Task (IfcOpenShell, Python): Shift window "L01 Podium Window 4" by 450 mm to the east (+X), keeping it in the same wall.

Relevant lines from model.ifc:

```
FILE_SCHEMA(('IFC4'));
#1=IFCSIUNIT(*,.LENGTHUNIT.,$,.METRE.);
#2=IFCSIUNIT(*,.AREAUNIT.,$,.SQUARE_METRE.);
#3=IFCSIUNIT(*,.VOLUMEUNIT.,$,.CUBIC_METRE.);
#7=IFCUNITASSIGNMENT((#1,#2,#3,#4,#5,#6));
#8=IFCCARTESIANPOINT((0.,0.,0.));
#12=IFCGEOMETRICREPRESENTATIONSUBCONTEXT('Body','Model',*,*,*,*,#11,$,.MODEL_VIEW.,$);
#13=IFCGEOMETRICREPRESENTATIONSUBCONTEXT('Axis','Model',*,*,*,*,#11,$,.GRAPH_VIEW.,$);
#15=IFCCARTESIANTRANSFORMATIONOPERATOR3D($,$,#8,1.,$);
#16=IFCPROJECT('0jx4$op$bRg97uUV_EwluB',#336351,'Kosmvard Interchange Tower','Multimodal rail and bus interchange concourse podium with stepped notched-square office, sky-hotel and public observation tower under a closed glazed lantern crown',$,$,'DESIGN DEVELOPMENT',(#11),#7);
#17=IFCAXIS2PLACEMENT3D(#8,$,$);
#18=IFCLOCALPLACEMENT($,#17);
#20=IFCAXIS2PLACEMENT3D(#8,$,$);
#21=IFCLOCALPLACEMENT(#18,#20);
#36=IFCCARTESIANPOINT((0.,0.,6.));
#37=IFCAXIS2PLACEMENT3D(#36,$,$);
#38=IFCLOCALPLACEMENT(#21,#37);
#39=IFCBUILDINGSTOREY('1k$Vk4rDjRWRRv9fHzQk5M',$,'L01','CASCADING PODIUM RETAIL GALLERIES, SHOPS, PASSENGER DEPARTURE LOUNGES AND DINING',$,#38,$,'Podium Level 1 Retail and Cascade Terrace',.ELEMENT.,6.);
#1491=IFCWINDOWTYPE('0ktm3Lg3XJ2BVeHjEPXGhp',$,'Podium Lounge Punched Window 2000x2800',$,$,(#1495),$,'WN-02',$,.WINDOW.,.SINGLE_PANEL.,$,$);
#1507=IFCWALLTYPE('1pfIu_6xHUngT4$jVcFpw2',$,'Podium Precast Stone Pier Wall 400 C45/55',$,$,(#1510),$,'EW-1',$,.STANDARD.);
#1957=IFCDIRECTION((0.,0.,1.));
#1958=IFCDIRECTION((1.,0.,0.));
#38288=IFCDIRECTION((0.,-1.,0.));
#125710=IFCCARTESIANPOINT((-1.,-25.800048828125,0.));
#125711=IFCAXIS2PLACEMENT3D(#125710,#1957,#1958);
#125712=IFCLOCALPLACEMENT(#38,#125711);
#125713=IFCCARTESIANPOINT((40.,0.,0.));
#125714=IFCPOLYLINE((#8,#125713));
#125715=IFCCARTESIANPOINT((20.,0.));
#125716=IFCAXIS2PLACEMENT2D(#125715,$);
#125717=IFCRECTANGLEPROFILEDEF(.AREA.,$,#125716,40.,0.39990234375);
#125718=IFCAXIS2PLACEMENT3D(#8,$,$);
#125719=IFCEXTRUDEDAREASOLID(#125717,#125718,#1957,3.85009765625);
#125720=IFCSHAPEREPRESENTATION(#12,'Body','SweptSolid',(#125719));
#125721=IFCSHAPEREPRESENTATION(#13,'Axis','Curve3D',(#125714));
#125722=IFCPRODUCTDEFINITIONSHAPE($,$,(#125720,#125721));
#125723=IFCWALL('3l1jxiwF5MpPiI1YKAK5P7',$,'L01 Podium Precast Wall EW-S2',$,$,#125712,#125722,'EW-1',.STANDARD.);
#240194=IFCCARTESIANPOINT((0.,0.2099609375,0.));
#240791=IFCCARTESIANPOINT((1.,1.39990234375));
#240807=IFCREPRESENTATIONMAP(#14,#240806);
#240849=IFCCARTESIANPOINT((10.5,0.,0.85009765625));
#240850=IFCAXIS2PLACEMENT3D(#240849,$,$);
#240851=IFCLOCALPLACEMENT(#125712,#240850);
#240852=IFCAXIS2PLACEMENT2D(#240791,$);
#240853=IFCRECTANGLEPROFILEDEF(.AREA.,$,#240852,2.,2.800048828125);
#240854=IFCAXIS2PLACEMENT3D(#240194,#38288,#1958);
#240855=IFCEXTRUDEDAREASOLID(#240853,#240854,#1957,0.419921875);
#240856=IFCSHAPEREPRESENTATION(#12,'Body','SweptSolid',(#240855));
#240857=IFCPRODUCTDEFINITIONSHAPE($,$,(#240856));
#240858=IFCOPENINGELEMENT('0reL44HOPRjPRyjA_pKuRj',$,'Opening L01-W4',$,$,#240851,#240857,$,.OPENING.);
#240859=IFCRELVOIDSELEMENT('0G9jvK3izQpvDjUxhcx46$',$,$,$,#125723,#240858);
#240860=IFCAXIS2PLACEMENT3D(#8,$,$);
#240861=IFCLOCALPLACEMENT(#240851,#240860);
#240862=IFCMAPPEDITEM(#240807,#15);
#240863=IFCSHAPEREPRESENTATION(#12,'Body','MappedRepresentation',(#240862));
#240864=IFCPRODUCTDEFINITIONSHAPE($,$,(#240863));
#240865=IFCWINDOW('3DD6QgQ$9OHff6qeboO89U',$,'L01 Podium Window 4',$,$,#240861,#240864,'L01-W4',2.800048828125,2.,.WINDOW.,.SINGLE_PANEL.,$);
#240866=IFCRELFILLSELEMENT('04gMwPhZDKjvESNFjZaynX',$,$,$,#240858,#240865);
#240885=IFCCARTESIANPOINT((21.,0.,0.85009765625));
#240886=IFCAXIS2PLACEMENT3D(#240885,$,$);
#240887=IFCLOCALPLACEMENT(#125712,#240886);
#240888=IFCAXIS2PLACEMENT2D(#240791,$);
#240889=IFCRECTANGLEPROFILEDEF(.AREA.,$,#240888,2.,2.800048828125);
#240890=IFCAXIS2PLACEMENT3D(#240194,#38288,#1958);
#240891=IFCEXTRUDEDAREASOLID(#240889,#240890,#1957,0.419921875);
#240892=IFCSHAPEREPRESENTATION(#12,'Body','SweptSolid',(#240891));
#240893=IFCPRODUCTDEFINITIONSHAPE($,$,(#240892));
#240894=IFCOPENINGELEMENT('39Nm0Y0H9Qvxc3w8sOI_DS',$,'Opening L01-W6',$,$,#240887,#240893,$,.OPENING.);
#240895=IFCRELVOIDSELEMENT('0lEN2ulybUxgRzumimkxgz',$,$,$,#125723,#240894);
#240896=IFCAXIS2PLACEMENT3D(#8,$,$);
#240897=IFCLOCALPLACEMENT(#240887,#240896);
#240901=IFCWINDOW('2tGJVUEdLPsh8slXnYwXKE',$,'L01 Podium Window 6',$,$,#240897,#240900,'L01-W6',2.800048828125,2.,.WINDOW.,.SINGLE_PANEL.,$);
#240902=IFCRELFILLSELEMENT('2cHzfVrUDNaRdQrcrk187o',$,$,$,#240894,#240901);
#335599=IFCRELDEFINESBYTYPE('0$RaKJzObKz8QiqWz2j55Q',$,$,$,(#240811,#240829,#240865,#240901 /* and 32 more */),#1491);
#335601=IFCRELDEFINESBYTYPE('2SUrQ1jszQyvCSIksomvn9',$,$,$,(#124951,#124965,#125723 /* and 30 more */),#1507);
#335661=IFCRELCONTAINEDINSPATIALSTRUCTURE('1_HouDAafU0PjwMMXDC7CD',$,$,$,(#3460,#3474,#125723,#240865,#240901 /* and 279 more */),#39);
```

```python
import ifcopenshell
import ifcopenshell.api.geometry
import ifcopenshell.util.placement

model = ifcopenshell.open("model.ifc")

window = model.by_guid("3DD6QgQ$9OHff6qeboO89U")
opening = window.FillsVoids[0].RelatingOpeningElement
wall = opening.VoidsElements[0].RelatingBuildingElement

wall_matrix = ifcopenshell.util.placement.get_local_placement(wall.ObjectPlacement)
shift = wall_matrix[:3, 0] * 0.45
before = ifcopenshell.util.placement.get_local_placement(window.ObjectPlacement)[:3, 3].copy()

# The window is placed relative to its opening, so it follows when the opening moves.
matrix = ifcopenshell.util.placement.get_local_placement(opening.ObjectPlacement)
matrix[:3, 3] += shift
ifcopenshell.api.geometry.edit_object_placement(
    model, product=opening, matrix=matrix, is_si=False, should_transform_children=True
)

after = ifcopenshell.util.placement.get_local_placement(window.ObjectPlacement)[:3, 3]
print("window moved by", (after - before).round(3) + 0.0)

model.write("model_rev.ifc")
```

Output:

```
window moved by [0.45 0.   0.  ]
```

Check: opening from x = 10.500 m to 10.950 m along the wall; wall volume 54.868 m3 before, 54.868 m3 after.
